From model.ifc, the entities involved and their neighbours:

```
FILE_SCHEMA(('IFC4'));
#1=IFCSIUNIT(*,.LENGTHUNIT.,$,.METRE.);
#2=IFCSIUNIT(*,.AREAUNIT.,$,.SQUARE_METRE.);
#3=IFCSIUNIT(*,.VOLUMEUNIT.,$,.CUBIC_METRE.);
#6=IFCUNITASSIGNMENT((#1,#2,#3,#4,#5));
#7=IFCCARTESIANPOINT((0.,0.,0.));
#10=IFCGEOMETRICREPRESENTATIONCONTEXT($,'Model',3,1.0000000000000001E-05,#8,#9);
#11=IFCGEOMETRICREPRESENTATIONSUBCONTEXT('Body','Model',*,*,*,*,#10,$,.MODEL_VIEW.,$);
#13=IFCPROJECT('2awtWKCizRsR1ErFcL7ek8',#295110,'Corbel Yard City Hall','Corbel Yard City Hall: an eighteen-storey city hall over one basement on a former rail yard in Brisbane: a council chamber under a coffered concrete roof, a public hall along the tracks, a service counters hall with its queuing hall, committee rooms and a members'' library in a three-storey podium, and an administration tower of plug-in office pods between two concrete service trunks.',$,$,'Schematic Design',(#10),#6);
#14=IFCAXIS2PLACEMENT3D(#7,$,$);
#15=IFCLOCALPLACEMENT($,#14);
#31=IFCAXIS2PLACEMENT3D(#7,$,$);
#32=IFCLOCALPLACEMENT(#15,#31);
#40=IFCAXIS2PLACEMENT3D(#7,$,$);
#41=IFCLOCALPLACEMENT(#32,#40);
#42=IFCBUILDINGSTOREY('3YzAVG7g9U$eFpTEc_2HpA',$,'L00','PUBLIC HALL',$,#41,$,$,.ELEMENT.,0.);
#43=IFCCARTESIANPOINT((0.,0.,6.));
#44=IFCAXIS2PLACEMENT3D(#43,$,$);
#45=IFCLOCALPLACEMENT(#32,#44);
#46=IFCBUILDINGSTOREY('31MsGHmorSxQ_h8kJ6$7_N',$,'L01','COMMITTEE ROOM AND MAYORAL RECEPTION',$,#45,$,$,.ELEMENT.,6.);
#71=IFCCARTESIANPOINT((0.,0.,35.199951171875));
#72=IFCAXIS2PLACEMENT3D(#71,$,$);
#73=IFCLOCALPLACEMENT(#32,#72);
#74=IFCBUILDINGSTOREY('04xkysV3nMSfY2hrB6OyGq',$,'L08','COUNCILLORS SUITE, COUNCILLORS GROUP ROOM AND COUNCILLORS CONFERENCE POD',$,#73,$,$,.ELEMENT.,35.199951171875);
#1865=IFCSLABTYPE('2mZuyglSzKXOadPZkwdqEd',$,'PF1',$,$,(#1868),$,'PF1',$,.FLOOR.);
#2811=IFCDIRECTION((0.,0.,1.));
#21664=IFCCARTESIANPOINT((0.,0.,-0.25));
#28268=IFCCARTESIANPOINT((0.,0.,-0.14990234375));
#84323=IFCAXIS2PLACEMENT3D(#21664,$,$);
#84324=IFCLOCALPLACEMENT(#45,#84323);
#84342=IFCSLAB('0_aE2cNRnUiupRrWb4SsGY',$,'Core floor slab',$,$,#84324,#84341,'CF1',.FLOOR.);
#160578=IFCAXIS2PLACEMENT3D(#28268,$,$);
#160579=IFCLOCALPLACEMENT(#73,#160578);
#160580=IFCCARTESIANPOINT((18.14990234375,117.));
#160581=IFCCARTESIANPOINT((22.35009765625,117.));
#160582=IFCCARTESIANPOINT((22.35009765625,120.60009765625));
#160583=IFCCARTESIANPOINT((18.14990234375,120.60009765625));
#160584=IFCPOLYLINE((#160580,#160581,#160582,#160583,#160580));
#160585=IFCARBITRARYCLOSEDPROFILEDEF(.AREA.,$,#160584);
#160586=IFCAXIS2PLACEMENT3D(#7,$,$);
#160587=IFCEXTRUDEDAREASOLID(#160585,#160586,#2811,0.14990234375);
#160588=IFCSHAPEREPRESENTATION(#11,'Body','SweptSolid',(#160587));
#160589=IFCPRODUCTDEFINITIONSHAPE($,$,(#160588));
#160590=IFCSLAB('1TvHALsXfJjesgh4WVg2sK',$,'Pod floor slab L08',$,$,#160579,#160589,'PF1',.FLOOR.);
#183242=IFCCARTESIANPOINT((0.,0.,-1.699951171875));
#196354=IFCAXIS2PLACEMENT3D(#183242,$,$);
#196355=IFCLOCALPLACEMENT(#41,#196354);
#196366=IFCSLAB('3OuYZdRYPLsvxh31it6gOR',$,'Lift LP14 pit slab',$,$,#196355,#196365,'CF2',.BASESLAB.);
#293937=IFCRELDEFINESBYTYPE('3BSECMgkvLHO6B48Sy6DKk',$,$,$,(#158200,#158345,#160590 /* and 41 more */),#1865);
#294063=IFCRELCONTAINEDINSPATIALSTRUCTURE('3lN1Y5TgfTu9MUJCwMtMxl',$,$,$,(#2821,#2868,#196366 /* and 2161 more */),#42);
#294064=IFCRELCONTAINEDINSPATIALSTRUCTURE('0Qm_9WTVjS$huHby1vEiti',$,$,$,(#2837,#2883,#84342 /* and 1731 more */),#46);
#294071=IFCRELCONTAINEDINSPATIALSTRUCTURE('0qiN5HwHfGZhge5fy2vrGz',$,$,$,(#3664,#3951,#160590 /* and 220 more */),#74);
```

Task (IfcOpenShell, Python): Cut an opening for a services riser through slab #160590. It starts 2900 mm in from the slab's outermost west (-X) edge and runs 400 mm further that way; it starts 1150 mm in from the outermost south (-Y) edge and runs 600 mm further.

```python
import numpy as np
import ifcopenshell
import ifcopenshell.api.feature
import ifcopenshell.api.geometry
import ifcopenshell.api.root
import ifcopenshell.geom
import ifcopenshell.util.placement
import ifcopenshell.util.representation
import ifcopenshell.util.shape
import ifcopenshell.util.unit

model = ifcopenshell.open("model.ifc")
unit_scale = ifcopenshell.util.unit.calculate_unit_scale(model)
settings = ifcopenshell.geom.settings()


def volume(element):
    """Net volume in cubic metres, openings subtracted."""
    shape = ifcopenshell.geom.create_shape(settings, element)
    return ifcopenshell.util.shape.get_volume(shape.geometry)


slab = model.by_id(160590)
before = volume(slab)

# Extent in the slab's own axes, in metres. The edges named are its -X and -Y sides.
slab_shape = ifcopenshell.geom.create_shape(settings, slab)
vertices = ifcopenshell.util.shape.get_vertices(slab_shape.geometry)
x_min, y_min, bottom = vertices.min(axis=0)
top = vertices[:, 2].max()

opening = ifcopenshell.api.root.create_entity(model, ifc_class="IfcOpeningElement", name="Services riser opening", predefined_type="OPENING")
context = ifcopenshell.util.representation.get_context(model, "Model", "Body", "MODEL_VIEW")
width, depth = 0.4, 0.6
outline = [(0.0, 0.0), (width, 0.0), (width, depth), (0.0, depth), (0.0, 0.0)]
# Overshoot both faces by 50 mm so the cut is clean.
shape = ifcopenshell.api.geometry.add_slab_representation(
    model, context=context, depth=top - bottom + 0.1, polyline=outline
)
ifcopenshell.api.geometry.assign_representation(model, product=opening, representation=shape)

matrix = ifcopenshell.util.placement.get_local_placement(slab.ObjectPlacement)
matrix[:, 3] = matrix @ np.append(np.array([x_min + 2.9, y_min + 1.15, bottom - 0.05]) / unit_scale, 1.0)
ifcopenshell.api.geometry.edit_object_placement(model, product=opening, matrix=matrix, is_si=False)
ifcopenshell.api.feature.add_feature(model, feature=opening, element=slab)

after = volume(slab)

print(f"slab volume {before:.3f} -> {after:.3f} m3")

model.write("model_updated.ifc")
```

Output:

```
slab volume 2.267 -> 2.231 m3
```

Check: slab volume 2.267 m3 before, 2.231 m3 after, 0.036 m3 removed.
